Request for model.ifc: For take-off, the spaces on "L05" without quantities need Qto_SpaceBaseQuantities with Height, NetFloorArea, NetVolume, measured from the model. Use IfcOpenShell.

First a look at what the model holds.

```python
import ifcopenshell
import ifcopenshell.util.element
import ifcopenshell.util.unit

model = ifcopenshell.open("model.ifc")
print(model.schema)
for unit_type in ("LENGTHUNIT", "AREAUNIT", "VOLUMEUNIT"):
    print(unit_type, ifcopenshell.util.unit.calculate_unit_scale(model, unit_type))
storey = next(s for s in model.by_type("IfcBuildingStorey") if s.Name == "L05")
spaces = [e for e in ifcopenshell.util.element.get_decomposition(storey) if e.is_a("IfcSpace")]
for e in sorted(spaces, key=lambda e: e.id()):
    print(e.id(), e.is_a(), e.Name, list(ifcopenshell.util.element.get_psets(e, qtos_only=True)), sep=" | ")
```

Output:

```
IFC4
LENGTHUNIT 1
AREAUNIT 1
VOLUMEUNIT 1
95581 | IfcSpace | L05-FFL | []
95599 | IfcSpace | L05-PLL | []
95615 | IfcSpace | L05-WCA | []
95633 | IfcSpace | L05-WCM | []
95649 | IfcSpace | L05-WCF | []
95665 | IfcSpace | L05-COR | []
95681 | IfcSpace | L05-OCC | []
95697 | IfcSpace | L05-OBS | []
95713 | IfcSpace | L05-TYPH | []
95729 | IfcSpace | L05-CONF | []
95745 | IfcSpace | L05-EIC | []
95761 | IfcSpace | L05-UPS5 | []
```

```python
import ifcopenshell
import ifcopenshell.api.pset
import ifcopenshell.geom
import ifcopenshell.util.element
import ifcopenshell.util.shape
import ifcopenshell.util.unit

model = ifcopenshell.open("model.ifc")
unit_scale = ifcopenshell.util.unit.calculate_unit_scale(model)
area_scale = ifcopenshell.util.unit.calculate_unit_scale(model, "AREAUNIT")
volume_scale = ifcopenshell.util.unit.calculate_unit_scale(model, "VOLUMEUNIT")
settings = ifcopenshell.geom.settings()

storey = next(s for s in model.by_type("IfcBuildingStorey") if s.Name == "L05")
spaces = [e for e in ifcopenshell.util.element.get_decomposition(storey) if e.is_a("IfcSpace")]

for e in sorted(spaces, key=lambda e: e.id()):
    if ifcopenshell.util.element.get_psets(e, qtos_only=True, should_inherit=False):
        continue
    # Geometry comes back in metres, in the element's own axes.
    shape = ifcopenshell.geom.create_shape(settings, e)
    values = {
        "Height": ifcopenshell.util.shape.get_z(shape.geometry) / unit_scale,
        "NetFloorArea": ifcopenshell.util.shape.get_footprint_area(shape.geometry) / area_scale,
        "NetVolume": ifcopenshell.util.shape.get_volume(shape.geometry) / volume_scale,
    }
    qto = ifcopenshell.api.pset.add_qto(model, product=e, name="Qto_SpaceBaseQuantities")
    ifcopenshell.api.pset.edit_qto(model, qto=qto, properties=values)
    print(e.id(), {k: round(v, 3) for k, v in values.items()})

model.write("model-out.ifc")
```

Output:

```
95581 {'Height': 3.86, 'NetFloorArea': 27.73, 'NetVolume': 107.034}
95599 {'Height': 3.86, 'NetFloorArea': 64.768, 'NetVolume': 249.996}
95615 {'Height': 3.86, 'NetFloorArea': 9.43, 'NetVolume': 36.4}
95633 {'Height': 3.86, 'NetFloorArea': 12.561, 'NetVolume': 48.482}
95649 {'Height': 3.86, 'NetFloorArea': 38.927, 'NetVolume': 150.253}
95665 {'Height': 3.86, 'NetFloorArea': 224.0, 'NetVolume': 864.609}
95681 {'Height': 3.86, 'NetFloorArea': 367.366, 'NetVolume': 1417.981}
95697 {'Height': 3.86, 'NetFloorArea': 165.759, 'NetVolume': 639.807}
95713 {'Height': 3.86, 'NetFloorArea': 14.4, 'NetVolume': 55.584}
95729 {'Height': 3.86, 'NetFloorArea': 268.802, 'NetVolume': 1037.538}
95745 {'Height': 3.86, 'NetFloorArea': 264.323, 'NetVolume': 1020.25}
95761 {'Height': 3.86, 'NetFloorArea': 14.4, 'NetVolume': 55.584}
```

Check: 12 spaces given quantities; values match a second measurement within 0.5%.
